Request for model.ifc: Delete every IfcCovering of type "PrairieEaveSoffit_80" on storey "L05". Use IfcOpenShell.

First a look at what the model holds.

```python
import ifcopenshell
import ifcopenshell.util.element

model = ifcopenshell.open("model.ifc")
print(model.schema)
storey = next(s for s in model.by_type("IfcBuildingStorey") if s.Name == "L05")
coverings = [e for e in ifcopenshell.util.element.get_decomposition(storey) if e.is_a("IfcCovering")]
seen = {}
for e in coverings:
    element_type = ifcopenshell.util.element.get_type(e)
    name = element_type.Name if element_type not in (None, e) else None
    seen[name] = seen.get(name, 0) + 1
for name, count in sorted(seen.items(), key=str):
    print(count, "x", name)
```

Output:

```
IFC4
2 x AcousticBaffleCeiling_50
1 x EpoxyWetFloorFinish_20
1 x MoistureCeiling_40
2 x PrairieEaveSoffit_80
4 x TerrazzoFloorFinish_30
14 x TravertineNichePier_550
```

```python
import ifcopenshell
import ifcopenshell.api.root
import ifcopenshell.util.element

model = ifcopenshell.open("model.ifc")

storey = next(s for s in model.by_type("IfcBuildingStorey") if s.Name == "L05")
coverings = [e for e in ifcopenshell.util.element.get_decomposition(storey) if e.is_a("IfcCovering")]
targets = [e for e in coverings if (t := ifcopenshell.util.element.get_type(e)) not in (None, e) and t.Name == "PrairieEaveSoffit_80"]

for e in targets:
    ifcopenshell.api.root.remove_product(model, product=e)
print(len(targets), "removed")

model.write("model_updated.ifc")
```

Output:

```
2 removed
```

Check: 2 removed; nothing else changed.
